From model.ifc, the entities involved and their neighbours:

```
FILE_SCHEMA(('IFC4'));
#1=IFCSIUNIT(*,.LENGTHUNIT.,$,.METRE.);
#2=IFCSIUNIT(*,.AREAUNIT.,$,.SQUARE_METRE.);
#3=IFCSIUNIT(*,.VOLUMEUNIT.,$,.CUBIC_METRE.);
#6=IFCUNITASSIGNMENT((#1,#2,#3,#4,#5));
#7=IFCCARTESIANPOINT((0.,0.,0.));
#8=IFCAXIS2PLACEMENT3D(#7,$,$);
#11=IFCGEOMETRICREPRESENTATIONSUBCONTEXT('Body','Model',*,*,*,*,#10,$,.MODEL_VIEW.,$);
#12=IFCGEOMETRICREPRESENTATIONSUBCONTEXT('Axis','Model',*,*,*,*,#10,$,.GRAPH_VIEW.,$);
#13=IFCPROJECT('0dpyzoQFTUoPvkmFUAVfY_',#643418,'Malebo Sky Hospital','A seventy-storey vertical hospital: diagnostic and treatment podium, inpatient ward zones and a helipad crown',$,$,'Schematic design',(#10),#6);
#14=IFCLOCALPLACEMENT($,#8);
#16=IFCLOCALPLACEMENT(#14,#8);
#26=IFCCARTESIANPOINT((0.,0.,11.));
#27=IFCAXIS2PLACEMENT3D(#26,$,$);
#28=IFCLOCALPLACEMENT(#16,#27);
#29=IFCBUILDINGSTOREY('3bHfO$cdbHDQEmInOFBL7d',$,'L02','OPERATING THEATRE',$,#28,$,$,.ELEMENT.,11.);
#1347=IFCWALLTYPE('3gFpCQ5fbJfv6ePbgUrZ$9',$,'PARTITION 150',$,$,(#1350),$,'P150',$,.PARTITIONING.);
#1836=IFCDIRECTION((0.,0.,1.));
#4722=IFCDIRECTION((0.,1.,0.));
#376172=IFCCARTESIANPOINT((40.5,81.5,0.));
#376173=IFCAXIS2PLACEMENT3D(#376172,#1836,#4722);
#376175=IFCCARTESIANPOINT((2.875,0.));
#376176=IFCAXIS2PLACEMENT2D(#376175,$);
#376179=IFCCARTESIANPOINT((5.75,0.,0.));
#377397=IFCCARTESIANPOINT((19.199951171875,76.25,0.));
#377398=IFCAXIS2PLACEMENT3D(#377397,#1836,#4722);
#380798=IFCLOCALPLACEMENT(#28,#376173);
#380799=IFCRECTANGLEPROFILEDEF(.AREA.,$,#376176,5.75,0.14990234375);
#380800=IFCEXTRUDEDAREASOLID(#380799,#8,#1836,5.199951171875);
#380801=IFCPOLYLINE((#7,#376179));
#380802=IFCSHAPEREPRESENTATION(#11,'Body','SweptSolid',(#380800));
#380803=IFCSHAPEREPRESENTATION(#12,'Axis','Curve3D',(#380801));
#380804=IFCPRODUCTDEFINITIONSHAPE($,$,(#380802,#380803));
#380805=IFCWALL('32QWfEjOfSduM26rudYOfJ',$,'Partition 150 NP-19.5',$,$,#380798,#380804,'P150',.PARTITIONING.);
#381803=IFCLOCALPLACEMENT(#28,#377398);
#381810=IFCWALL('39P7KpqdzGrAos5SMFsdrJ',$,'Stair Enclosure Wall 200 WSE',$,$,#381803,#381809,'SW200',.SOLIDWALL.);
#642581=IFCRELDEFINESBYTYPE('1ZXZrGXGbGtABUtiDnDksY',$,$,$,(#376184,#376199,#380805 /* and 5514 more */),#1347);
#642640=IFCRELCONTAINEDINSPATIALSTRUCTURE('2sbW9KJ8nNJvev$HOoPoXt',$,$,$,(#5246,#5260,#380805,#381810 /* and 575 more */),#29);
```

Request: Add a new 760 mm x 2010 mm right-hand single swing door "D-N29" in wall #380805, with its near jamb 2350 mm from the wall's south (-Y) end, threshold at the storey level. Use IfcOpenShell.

```python
import numpy as np
import ifcopenshell
import ifcopenshell.api.feature
import ifcopenshell.api.geometry
import ifcopenshell.api.root
import ifcopenshell.api.spatial
import ifcopenshell.geom
import ifcopenshell.util.element
import ifcopenshell.util.placement
import ifcopenshell.util.representation
import ifcopenshell.util.shape
import ifcopenshell.util.unit

model = ifcopenshell.open("model.ifc")
unit_scale = ifcopenshell.util.unit.calculate_unit_scale(model)
settings = ifcopenshell.geom.settings()


def volume(element):
    """Net volume in cubic metres, openings subtracted."""
    shape = ifcopenshell.geom.create_shape(settings, element)
    return ifcopenshell.util.shape.get_volume(shape.geometry)


wall = model.by_guid("32QWfEjOfSduM26rudYOfJ")
storey = ifcopenshell.util.element.get_container(wall, ifc_class="IfcBuildingStorey")
context = ifcopenshell.util.representation.get_context(model, "Model", "Body", "MODEL_VIEW")
before = volume(wall)

width, height, from_end, sill = 0.76, 2.01, 2.35, 0.0  # metres

# The wall runs along its own X axis, and the end named is its -X end.
wall_shape = ifcopenshell.geom.create_shape(settings, wall)
x, y, z = ifcopenshell.util.shape.get_vertices(wall_shape.geometry).T
start = x.min() + from_end
face, thickness = float(y.min()), float(y.max() - y.min())
wall_matrix = ifcopenshell.util.placement.get_local_placement(wall.ObjectPlacement)
level = ifcopenshell.util.placement.get_local_placement(storey.ObjectPlacement)[2, 3]


def in_wall(x, y):
    """Placement at x, y metres in the wall's axes, at sill height."""
    matrix = wall_matrix.copy()
    matrix[:, 3] = wall_matrix @ np.array([x / unit_scale, y / unit_scale, 0.0, 1.0])
    matrix[2, 3] = level + sill / unit_scale
    return matrix


# Opening: a box that overshoots both wall faces by 50 mm.
opening = ifcopenshell.api.root.create_entity(model, ifc_class="IfcOpeningElement", predefined_type="OPENING")
box = ifcopenshell.api.geometry.add_wall_representation(
    model, context=context, length=width, height=height, thickness=thickness + 0.1
)
ifcopenshell.api.geometry.assign_representation(model, product=opening, representation=box)
ifcopenshell.api.geometry.edit_object_placement(model, product=opening, matrix=in_wall(start, face - 0.05), is_si=False)
ifcopenshell.api.feature.add_feature(model, feature=opening, element=wall)

door = ifcopenshell.api.root.create_entity(model, ifc_class="IfcDoor", name="D-N29", predefined_type="DOOR")
door.OverallWidth, door.OverallHeight = width / unit_scale, height / unit_scale
door.OperationType = "SINGLE_SWING_RIGHT"
body = ifcopenshell.api.geometry.add_door_representation(
    model,
    context=context,
    overall_width=door.OverallWidth,
    overall_height=door.OverallHeight,
    operation_type="SINGLE_SWING_RIGHT",
    lining_properties={"LiningDepth": thickness / unit_scale, "ThresholdDepth": thickness / unit_scale},
)
ifcopenshell.api.geometry.assign_representation(model, product=door, representation=body)
ifcopenshell.api.spatial.assign_container(model, products=[door], relating_structure=storey)
ifcopenshell.api.feature.add_filling(model, opening=opening, element=door)

# The lining spans the wall, so the door starts at the wall face.
ifcopenshell.api.geometry.edit_object_placement(model, product=door, matrix=in_wall(start, face), is_si=False)

after = volume(wall)

print(f"wall volume {before:.3f} -> {after:.3f} m3")

model.write("model_updated.ifc")
```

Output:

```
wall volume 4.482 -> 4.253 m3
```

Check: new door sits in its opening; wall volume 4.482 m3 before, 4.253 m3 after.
